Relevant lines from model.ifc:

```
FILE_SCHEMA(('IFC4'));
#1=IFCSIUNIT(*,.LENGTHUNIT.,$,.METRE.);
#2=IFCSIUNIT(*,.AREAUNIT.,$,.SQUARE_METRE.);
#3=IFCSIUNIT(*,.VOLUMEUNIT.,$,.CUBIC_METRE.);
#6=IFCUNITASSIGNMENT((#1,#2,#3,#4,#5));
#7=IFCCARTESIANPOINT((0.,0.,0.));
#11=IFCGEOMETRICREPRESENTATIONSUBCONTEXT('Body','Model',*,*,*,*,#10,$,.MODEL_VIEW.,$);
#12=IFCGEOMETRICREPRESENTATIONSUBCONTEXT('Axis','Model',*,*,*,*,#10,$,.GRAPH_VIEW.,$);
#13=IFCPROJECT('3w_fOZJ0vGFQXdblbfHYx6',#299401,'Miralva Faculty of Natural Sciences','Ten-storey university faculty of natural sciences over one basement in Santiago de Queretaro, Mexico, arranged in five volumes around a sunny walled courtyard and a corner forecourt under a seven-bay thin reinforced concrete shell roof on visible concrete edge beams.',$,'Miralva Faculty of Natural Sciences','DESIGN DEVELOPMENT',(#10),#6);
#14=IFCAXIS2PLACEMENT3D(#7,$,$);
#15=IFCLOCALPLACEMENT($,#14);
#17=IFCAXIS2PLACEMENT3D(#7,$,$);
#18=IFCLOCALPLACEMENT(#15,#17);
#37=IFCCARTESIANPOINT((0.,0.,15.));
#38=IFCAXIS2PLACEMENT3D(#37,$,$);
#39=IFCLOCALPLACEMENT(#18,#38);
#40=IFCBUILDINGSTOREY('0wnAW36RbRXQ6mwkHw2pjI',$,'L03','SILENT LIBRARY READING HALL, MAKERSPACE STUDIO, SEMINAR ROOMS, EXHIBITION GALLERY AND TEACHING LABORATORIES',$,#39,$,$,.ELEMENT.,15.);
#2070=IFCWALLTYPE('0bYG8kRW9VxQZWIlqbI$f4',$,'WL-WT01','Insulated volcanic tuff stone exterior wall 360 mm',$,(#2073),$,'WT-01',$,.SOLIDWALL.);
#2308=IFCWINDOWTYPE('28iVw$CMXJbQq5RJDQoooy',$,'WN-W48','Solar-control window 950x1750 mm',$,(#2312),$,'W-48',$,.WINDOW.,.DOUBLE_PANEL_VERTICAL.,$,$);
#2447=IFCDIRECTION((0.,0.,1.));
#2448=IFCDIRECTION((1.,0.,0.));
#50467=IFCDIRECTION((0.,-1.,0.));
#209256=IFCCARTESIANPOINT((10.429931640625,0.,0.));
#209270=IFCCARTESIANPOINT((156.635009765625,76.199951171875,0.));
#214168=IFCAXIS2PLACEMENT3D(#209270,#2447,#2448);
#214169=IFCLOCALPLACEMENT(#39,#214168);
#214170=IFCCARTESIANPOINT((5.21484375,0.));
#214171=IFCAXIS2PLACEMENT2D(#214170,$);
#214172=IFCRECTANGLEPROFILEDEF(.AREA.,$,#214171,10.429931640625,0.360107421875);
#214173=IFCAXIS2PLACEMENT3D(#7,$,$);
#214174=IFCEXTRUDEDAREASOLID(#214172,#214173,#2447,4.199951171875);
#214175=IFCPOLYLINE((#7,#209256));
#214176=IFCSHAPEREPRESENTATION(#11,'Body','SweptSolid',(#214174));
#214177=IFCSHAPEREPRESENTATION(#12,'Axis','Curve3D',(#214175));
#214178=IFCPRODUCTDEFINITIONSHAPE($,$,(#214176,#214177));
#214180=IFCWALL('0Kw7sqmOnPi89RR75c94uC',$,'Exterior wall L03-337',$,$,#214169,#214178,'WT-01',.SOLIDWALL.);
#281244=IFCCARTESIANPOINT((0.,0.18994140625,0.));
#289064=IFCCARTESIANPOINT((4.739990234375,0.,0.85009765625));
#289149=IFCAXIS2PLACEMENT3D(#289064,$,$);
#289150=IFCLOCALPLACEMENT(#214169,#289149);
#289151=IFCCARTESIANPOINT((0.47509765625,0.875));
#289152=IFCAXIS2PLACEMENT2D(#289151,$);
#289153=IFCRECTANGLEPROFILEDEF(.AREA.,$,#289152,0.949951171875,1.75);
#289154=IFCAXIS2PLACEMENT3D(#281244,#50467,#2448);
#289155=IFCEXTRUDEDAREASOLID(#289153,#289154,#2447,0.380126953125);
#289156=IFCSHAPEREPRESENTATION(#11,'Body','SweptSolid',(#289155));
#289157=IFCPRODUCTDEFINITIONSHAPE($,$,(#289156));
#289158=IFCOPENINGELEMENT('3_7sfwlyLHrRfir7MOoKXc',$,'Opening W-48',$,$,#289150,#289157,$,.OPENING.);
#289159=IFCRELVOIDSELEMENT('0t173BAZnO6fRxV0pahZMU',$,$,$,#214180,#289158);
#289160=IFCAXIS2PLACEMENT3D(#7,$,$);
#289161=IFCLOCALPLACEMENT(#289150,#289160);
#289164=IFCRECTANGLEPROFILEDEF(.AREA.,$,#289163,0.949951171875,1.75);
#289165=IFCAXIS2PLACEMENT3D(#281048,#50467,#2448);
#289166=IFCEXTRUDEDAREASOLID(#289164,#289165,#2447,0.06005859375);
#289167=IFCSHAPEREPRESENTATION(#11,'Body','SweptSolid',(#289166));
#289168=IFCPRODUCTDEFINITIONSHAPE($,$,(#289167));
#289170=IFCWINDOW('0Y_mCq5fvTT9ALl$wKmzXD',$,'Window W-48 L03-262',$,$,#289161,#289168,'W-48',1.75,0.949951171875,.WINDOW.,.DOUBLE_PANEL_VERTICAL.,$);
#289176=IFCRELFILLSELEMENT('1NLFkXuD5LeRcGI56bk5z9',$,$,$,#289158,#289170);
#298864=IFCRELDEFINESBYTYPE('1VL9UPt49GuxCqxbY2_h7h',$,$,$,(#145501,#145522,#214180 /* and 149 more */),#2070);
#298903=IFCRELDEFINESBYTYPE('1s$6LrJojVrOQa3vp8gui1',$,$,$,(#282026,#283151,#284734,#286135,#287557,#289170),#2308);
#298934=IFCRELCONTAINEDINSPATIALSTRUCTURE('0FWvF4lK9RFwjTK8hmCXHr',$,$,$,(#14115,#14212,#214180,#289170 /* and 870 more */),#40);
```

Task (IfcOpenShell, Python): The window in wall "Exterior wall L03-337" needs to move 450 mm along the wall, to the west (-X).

```python
import ifcopenshell
import ifcopenshell.api.geometry
import ifcopenshell.util.placement
import ifcopenshell.util.unit

model = ifcopenshell.open("model.ifc")
unit_scale = ifcopenshell.util.unit.calculate_unit_scale(model)

window = model.by_id(289170)
opening = window.FillsVoids[0].RelatingOpeningElement
wall = opening.VoidsElements[0].RelatingBuildingElement

wall_matrix = ifcopenshell.util.placement.get_local_placement(wall.ObjectPlacement)
shift = wall_matrix[:3, 0] * -0.45 / unit_scale
before = ifcopenshell.util.placement.get_local_placement(window.ObjectPlacement)[:3, 3].copy()

# The window is placed relative to its opening, so it follows when the opening moves.
matrix = ifcopenshell.util.placement.get_local_placement(opening.ObjectPlacement)
matrix[:3, 3] += shift
ifcopenshell.api.geometry.edit_object_placement(
    model, product=opening, matrix=matrix, is_si=False, should_transform_children=True
)

after = ifcopenshell.util.placement.get_local_placement(window.ObjectPlacement)[:3, 3]
print("window moved by", (after - before).round(3) + 0.0)

model.write("model_updated.ifc")
```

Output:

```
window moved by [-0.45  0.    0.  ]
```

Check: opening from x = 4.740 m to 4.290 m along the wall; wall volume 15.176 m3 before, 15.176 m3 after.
